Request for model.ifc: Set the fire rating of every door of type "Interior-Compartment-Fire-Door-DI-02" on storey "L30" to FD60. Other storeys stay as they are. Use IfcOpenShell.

First a look at what the model holds.

```python
import ifcopenshell
import ifcopenshell.util.element

model = ifcopenshell.open("model.ifc")
print(model.schema)
storey = next(s for s in model.by_type("IfcBuildingStorey") if s.Name == "L30")
doors = [e for e in ifcopenshell.util.element.get_decomposition(storey) if e.is_a("IfcDoor")]
seen = {}
for e in doors:
    element_type = ifcopenshell.util.element.get_type(e)
    key = (element_type.Name if element_type != e and element_type else None, ifcopenshell.util.element.get_pset(e, "Pset_DoorCommon", "FireRating"))
    seen[key] = seen.get(key, 0) + 1
for (name, value), count in sorted(seen.items(), key=str):
    print(count, "x", name, "|", value)
```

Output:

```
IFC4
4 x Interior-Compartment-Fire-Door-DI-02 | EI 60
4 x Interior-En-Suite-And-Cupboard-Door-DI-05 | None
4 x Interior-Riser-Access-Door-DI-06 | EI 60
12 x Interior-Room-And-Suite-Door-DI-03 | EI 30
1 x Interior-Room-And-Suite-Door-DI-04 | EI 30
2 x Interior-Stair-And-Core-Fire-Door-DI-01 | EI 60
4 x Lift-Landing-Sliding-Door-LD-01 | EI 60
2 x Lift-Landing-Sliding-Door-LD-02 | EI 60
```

```python
import ifcopenshell
import ifcopenshell.api.pset
import ifcopenshell.util.element

model = ifcopenshell.open("model.ifc")

storey = next(s for s in model.by_type("IfcBuildingStorey") if s.Name == "L30")
doors = [e for e in ifcopenshell.util.element.get_decomposition(storey) if e.is_a("IfcDoor")]

count = 0
for e in doors:
    element_type = ifcopenshell.util.element.get_type(e)
    if element_type in (None, e) or element_type.Name != "Interior-Compartment-Fire-Door-DI-02":
        continue
    found = ifcopenshell.util.element.get_pset(e, "Pset_DoorCommon", should_inherit=False)
    if found:
        pset = model.by_id(found["id"])
        if len(ifcopenshell.util.element.get_elements_by_pset(pset)) > 1:
            pset = ifcopenshell.api.pset.unshare_pset(model, products=[e], pset=pset)[0]
    else:
        pset = ifcopenshell.api.pset.add_pset(model, product=e, name="Pset_DoorCommon")
    ifcopenshell.api.pset.edit_pset(model, pset=pset, properties={"FireRating": "FD60"})
    count += 1

print(count, "doors updated")

model.write("model_rev.ifc")
```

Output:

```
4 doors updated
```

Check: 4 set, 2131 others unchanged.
